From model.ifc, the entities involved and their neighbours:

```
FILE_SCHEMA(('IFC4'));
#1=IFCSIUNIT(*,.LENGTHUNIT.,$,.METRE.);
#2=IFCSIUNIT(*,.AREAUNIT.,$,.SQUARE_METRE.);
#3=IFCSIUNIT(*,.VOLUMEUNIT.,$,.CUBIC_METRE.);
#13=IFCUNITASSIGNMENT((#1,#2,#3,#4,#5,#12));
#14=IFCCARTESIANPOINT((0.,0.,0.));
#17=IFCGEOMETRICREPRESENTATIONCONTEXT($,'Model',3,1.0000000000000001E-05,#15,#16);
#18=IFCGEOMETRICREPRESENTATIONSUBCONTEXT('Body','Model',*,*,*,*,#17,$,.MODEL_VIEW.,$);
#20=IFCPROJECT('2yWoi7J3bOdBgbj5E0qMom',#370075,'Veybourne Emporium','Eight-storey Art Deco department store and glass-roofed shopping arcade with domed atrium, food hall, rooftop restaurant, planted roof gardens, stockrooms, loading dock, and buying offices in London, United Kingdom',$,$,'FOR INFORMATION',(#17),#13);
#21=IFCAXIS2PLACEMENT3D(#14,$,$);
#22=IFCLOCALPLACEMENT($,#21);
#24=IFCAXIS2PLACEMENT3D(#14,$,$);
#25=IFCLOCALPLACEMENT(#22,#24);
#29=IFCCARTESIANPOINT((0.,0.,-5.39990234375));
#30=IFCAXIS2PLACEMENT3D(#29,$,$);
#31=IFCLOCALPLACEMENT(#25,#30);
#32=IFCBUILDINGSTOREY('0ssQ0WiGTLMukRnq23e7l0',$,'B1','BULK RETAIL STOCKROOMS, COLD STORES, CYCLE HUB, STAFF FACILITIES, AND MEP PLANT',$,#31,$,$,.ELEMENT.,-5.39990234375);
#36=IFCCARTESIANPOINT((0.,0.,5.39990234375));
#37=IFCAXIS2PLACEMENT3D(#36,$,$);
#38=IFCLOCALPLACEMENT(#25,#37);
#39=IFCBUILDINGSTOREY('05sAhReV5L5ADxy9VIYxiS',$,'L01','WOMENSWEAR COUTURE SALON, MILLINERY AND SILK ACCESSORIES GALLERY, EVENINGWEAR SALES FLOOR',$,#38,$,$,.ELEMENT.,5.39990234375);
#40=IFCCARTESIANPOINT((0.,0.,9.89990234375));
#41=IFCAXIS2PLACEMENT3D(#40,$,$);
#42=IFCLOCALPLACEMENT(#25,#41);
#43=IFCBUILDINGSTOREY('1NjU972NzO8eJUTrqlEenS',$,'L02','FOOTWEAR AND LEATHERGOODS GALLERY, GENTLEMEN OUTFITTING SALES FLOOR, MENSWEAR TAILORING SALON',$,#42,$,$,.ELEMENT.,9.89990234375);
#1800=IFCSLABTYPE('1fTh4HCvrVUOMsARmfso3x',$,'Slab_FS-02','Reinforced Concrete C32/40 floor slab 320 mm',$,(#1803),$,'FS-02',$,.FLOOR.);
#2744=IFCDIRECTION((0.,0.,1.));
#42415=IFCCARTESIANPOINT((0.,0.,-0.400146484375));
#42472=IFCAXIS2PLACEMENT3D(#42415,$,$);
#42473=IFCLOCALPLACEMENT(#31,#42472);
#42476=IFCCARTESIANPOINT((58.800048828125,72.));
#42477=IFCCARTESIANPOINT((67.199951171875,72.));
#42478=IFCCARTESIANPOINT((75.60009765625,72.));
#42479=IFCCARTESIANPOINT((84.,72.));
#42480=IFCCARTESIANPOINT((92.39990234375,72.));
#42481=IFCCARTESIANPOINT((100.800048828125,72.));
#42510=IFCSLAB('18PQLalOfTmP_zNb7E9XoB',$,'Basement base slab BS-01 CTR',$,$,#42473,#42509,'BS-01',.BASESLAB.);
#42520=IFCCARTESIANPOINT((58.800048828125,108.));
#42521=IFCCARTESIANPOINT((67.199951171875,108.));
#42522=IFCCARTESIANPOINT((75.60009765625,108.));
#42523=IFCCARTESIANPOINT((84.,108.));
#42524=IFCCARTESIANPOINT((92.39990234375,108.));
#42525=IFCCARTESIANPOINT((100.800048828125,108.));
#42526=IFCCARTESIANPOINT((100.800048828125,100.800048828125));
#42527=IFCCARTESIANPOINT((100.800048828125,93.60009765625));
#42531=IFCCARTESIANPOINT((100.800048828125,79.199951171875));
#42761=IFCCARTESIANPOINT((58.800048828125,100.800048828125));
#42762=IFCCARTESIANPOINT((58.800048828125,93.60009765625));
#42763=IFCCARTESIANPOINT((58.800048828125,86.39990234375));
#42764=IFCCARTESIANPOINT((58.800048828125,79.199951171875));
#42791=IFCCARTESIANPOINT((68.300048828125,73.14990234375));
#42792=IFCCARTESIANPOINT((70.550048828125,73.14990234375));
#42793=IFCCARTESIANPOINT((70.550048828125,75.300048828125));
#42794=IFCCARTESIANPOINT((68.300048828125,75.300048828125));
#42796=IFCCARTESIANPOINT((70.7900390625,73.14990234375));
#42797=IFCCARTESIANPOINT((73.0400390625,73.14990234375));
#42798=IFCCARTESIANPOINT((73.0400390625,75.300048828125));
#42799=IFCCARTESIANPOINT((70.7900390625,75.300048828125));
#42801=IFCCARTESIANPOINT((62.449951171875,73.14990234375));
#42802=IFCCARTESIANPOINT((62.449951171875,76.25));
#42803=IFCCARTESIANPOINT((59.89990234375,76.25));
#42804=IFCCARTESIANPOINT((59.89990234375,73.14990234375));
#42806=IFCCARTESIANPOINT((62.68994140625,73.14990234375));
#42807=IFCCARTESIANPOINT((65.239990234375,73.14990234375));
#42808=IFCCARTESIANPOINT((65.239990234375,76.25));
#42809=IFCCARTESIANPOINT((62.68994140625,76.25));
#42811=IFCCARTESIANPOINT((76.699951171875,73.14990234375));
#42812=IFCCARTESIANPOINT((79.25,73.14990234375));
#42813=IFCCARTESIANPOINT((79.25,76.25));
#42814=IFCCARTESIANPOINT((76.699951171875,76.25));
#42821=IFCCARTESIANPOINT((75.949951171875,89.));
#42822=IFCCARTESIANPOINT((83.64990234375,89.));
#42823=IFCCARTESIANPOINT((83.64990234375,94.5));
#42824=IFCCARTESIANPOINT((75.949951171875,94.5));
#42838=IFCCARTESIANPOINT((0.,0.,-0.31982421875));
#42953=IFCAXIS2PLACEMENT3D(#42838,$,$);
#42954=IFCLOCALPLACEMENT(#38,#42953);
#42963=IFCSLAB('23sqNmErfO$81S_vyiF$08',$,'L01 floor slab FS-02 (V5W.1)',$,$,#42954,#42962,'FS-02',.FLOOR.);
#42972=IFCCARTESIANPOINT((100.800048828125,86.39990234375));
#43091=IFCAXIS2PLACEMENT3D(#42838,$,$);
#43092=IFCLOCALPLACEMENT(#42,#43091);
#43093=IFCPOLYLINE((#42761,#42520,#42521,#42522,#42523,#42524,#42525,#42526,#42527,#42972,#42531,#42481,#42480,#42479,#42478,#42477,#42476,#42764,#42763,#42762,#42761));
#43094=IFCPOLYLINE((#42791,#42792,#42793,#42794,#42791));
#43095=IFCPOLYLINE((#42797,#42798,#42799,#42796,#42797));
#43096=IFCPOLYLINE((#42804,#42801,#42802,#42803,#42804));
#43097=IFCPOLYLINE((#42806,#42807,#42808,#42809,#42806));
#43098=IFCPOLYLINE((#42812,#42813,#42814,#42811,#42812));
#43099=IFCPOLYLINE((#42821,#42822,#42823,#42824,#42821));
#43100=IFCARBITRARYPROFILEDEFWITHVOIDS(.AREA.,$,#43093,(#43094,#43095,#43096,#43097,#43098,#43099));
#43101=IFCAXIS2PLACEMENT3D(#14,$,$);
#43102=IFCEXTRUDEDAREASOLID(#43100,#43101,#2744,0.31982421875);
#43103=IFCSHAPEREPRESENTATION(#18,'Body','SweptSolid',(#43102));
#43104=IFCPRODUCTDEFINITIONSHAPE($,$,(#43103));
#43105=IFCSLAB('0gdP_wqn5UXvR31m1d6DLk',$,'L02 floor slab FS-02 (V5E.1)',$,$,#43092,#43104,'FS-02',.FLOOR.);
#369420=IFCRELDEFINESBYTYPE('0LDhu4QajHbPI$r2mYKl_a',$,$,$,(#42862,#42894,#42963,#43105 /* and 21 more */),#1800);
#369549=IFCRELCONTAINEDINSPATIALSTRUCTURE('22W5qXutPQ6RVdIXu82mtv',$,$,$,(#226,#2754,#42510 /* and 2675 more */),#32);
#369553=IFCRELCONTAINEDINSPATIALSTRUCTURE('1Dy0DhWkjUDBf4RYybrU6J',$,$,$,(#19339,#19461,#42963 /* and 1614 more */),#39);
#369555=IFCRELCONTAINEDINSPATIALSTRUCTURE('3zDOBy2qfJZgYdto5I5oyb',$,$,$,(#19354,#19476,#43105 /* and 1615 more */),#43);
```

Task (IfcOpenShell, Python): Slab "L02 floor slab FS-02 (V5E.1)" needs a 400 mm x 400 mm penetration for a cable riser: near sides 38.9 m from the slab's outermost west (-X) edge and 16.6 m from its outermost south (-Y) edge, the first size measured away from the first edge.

```python
import numpy as np
import ifcopenshell
import ifcopenshell.api.feature
import ifcopenshell.api.geometry
import ifcopenshell.api.root
import ifcopenshell.geom
import ifcopenshell.util.placement
import ifcopenshell.util.representation
import ifcopenshell.util.shape
import ifcopenshell.util.unit

model = ifcopenshell.open("model.ifc")
unit_scale = ifcopenshell.util.unit.calculate_unit_scale(model)
settings = ifcopenshell.geom.settings()


def volume(element):
    """Net volume in cubic metres, openings subtracted."""
    shape = ifcopenshell.geom.create_shape(settings, element)
    return ifcopenshell.util.shape.get_volume(shape.geometry)


slab = model.by_guid("0gdP_wqn5UXvR31m1d6DLk")
before = volume(slab)

# Extent in the slab's own axes, in metres. The edges named are its -X and -Y sides.
slab_shape = ifcopenshell.geom.create_shape(settings, slab)
vertices = ifcopenshell.util.shape.get_vertices(slab_shape.geometry)
x_min, y_min, bottom = vertices.min(axis=0)
top = vertices[:, 2].max()

opening = ifcopenshell.api.root.create_entity(model, ifc_class="IfcOpeningElement", name="Cable riser opening", predefined_type="OPENING")
context = ifcopenshell.util.representation.get_context(model, "Model", "Body", "MODEL_VIEW")
width, depth = 0.4, 0.4
outline = [(0.0, 0.0), (width, 0.0), (width, depth), (0.0, depth), (0.0, 0.0)]
# Overshoot both faces by 50 mm so the cut is clean.
shape = ifcopenshell.api.geometry.add_slab_representation(
    model, context=context, depth=top - bottom + 0.1, polyline=outline
)
ifcopenshell.api.geometry.assign_representation(model, product=opening, representation=shape)

matrix = ifcopenshell.util.placement.get_local_placement(slab.ObjectPlacement)
matrix[:, 3] = matrix @ np.append(np.array([x_min + 38.9, y_min + 16.6, bottom - 0.05]) / unit_scale, 1.0)
ifcopenshell.api.geometry.edit_object_placement(model, product=opening, matrix=matrix, is_si=False)
ifcopenshell.api.feature.add_feature(model, feature=opening, element=slab)

after = volume(slab)

print(f"slab volume {before:.3f} -> {after:.3f} m3")

model.write("model-out.ifc")
```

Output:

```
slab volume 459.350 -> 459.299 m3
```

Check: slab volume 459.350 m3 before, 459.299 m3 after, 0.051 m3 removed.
